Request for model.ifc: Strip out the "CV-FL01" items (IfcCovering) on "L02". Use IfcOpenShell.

First a look at what the model holds.

```python
import ifcopenshell
import ifcopenshell.util.element

model = ifcopenshell.open("model.ifc")
print(model.schema)
storey = next(s for s in model.by_type("IfcBuildingStorey") if s.Name == "L02")
coverings = [e for e in ifcopenshell.util.element.get_decomposition(storey) if e.is_a("IfcCovering")]
seen = {}
for e in coverings:
    element_type = ifcopenshell.util.element.get_type(e)
    name = element_type.Name if element_type not in (None, e) else None
    seen[name] = seen.get(name, 0) + 1
for name, count in sorted(seen.items(), key=str):
    print(count, "x", name)
```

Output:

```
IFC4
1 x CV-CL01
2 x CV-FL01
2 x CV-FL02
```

```python
import ifcopenshell
import ifcopenshell.api.root
import ifcopenshell.util.element

model = ifcopenshell.open("model.ifc")

storey = next(s for s in model.by_type("IfcBuildingStorey") if s.Name == "L02")
coverings = [e for e in ifcopenshell.util.element.get_decomposition(storey) if e.is_a("IfcCovering")]
targets = [e for e in coverings if (t := ifcopenshell.util.element.get_type(e)) not in (None, e) and t.Name == "CV-FL01"]

for e in targets:
    ifcopenshell.api.root.remove_product(model, product=e)
print(len(targets), "removed")

model.write("model_v2.ifc")
```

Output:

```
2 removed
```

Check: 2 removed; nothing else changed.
